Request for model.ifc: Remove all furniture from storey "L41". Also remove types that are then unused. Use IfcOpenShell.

First a look at what the model holds.

```python
import ifcopenshell
import ifcopenshell.util.element

model = ifcopenshell.open("model.ifc")
print(model.schema)
storey = next(s for s in model.by_type("IfcBuildingStorey") if s.Name == "L41")
furniture = [e for e in ifcopenshell.util.element.get_decomposition(storey) if e.is_a("IfcFurnishingElement")]
seen = {}
for e in furniture:
    element_type = ifcopenshell.util.element.get_type(e)
    name = element_type.Name if element_type not in (None, e) else None
    seen[name] = seen.get(name, 0) + 1
for name, count in sorted(seen.items(), key=str):
    print(count, "x", name)
```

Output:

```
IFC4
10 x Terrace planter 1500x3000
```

```python
import ifcopenshell
import ifcopenshell.api.root
import ifcopenshell.util.element

model = ifcopenshell.open("model.ifc")

storey = next(s for s in model.by_type("IfcBuildingStorey") if s.Name == "L41")
furniture = [e for e in ifcopenshell.util.element.get_decomposition(storey) if e.is_a("IfcFurnishingElement")]
types = {ifcopenshell.util.element.get_type(e) for e in furniture} - {None, *furniture}

for e in furniture:
    ifcopenshell.api.root.remove_product(model, product=e)
print(len(furniture), "removed")

unused = [t for t in types if not ifcopenshell.util.element.get_types(t)]
for t in unused:
    ifcopenshell.api.root.remove_product(model, product=t)
print(len(unused), "unused types removed")

model.write("model_v2.ifc")
```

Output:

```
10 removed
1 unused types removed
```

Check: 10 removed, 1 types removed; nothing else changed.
